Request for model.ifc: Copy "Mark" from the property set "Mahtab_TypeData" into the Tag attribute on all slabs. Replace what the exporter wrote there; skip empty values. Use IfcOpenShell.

First a look at what the model holds.

```python
import ifcopenshell
import ifcopenshell.util.element

model = ifcopenshell.open("model.ifc")
print(model.schema)
slabs = model.by_type("IfcSlab")
print(len(slabs), "slabs")
for e in slabs[:8]:
    source = ifcopenshell.util.element.get_pset(e, "Mahtab_TypeData", "Mark")
    target = e.Tag
    print(e.id(), repr(source), repr(target), sep=" | ")
```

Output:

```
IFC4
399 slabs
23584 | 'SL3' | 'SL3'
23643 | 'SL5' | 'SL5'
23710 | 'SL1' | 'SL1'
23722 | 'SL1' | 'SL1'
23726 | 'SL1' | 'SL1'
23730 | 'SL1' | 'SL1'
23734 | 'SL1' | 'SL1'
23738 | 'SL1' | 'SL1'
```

```python
import ifcopenshell
import ifcopenshell.util.element

model = ifcopenshell.open("model.ifc")

count = 0
for e in model.by_type("IfcSlab"):
    value = ifcopenshell.util.element.get_pset(e, "Mahtab_TypeData", "Mark")
    current = e.Tag
    if not value or not value.strip() or current == value:
        continue
    e.Tag = value
    count += 1

print(count, "slabs updated")

model.write("model_rev.ifc")
```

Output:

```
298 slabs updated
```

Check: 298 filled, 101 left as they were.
